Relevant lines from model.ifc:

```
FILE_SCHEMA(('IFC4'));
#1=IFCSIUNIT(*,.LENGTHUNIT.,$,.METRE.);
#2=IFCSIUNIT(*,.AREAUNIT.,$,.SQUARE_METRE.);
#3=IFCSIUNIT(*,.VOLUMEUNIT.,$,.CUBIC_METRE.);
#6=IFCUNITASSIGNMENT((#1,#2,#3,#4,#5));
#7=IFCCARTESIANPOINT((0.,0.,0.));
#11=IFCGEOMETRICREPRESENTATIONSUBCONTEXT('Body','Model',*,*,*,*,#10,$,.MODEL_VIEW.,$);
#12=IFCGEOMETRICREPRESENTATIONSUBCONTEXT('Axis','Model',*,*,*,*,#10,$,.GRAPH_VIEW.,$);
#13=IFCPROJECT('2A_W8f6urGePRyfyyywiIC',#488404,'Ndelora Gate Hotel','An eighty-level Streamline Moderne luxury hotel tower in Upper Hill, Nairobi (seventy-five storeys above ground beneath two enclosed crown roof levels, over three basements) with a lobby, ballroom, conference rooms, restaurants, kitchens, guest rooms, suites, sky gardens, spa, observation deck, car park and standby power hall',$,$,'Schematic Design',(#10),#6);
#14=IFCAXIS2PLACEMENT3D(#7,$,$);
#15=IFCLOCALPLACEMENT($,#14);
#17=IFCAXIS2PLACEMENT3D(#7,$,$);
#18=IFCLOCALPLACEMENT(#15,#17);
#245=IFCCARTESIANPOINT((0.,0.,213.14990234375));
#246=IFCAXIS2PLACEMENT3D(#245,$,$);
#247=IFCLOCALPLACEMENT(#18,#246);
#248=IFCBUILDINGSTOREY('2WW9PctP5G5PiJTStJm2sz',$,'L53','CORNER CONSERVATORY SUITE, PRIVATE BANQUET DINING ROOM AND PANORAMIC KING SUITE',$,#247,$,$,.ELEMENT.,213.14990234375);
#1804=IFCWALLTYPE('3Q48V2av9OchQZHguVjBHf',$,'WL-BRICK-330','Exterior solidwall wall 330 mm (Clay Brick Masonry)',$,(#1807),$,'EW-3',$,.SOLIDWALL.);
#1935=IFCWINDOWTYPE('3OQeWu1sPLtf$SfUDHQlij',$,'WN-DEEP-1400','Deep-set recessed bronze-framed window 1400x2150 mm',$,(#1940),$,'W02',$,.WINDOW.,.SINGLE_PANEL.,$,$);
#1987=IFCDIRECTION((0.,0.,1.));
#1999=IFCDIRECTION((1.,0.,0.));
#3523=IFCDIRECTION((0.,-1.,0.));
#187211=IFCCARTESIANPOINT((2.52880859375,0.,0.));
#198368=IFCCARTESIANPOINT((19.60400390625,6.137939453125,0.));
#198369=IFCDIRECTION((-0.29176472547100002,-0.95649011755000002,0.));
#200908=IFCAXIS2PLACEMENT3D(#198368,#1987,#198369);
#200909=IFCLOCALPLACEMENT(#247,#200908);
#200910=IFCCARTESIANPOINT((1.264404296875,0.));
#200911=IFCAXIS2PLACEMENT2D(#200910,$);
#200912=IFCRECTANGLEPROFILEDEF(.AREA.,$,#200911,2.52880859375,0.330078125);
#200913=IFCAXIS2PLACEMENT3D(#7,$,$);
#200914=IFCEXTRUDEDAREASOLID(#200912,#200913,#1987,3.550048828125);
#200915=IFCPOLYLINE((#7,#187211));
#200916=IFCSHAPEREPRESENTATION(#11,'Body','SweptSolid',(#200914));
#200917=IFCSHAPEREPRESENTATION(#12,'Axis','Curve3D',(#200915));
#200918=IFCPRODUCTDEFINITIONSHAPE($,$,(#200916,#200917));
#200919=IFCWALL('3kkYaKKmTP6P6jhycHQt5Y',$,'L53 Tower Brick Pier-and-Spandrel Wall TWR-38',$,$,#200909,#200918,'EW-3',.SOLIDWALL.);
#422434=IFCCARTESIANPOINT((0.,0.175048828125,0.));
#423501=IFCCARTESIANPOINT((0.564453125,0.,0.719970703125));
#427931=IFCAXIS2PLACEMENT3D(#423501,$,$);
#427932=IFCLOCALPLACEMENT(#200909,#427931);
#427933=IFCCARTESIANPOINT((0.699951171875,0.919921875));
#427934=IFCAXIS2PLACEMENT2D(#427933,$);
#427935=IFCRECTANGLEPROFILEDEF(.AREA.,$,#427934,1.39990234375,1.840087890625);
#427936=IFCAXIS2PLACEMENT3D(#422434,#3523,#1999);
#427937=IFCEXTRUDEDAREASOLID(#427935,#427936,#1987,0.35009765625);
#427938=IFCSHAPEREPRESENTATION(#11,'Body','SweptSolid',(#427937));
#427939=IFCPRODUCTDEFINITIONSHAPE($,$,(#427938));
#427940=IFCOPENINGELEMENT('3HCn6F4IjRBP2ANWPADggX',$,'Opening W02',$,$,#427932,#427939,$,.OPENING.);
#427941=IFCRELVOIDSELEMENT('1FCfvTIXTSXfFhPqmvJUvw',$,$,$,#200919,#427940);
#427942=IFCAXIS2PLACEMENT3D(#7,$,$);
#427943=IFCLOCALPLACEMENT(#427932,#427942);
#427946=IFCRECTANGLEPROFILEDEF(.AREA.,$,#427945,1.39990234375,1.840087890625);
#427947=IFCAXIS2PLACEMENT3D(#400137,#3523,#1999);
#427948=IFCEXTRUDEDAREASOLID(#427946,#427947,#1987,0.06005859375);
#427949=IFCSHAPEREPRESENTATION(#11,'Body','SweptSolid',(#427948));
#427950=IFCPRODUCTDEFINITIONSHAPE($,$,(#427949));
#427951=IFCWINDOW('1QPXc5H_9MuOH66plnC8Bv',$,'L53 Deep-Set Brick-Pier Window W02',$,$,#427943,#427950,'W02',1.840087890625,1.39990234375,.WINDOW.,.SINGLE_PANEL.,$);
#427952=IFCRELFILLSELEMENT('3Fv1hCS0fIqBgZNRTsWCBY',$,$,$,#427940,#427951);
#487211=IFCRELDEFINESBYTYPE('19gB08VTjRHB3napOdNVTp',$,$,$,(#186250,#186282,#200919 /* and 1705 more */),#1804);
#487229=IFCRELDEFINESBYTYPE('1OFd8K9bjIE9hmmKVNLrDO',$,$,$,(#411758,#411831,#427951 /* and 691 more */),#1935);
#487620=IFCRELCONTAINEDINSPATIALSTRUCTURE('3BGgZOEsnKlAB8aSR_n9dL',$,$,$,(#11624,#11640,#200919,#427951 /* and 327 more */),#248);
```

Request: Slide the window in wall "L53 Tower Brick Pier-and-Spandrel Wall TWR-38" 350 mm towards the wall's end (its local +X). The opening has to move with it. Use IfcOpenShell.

```python
import ifcopenshell
import ifcopenshell.api.geometry
import ifcopenshell.util.placement
import ifcopenshell.util.unit

model = ifcopenshell.open("model.ifc")
unit_scale = ifcopenshell.util.unit.calculate_unit_scale(model)

window = model.by_id(427951)
opening = window.FillsVoids[0].RelatingOpeningElement
wall = opening.VoidsElements[0].RelatingBuildingElement

wall_matrix = ifcopenshell.util.placement.get_local_placement(wall.ObjectPlacement)
shift = wall_matrix[:3, 0] * 0.35 / unit_scale
before = ifcopenshell.util.placement.get_local_placement(window.ObjectPlacement)[:3, 3].copy()

# The window is placed relative to its opening, so it follows when the opening moves.
matrix = ifcopenshell.util.placement.get_local_placement(opening.ObjectPlacement)
matrix[:3, 3] += shift
ifcopenshell.api.geometry.edit_object_placement(
    model, product=opening, matrix=matrix, is_si=False, should_transform_children=True
)

after = ifcopenshell.util.placement.get_local_placement(window.ObjectPlacement)[:3, 3]
print("window moved by", (after - before).round(3) + 0.0)

model.write("model-out.ifc")
```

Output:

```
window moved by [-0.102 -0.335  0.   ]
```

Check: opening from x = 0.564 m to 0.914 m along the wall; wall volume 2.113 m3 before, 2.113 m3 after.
